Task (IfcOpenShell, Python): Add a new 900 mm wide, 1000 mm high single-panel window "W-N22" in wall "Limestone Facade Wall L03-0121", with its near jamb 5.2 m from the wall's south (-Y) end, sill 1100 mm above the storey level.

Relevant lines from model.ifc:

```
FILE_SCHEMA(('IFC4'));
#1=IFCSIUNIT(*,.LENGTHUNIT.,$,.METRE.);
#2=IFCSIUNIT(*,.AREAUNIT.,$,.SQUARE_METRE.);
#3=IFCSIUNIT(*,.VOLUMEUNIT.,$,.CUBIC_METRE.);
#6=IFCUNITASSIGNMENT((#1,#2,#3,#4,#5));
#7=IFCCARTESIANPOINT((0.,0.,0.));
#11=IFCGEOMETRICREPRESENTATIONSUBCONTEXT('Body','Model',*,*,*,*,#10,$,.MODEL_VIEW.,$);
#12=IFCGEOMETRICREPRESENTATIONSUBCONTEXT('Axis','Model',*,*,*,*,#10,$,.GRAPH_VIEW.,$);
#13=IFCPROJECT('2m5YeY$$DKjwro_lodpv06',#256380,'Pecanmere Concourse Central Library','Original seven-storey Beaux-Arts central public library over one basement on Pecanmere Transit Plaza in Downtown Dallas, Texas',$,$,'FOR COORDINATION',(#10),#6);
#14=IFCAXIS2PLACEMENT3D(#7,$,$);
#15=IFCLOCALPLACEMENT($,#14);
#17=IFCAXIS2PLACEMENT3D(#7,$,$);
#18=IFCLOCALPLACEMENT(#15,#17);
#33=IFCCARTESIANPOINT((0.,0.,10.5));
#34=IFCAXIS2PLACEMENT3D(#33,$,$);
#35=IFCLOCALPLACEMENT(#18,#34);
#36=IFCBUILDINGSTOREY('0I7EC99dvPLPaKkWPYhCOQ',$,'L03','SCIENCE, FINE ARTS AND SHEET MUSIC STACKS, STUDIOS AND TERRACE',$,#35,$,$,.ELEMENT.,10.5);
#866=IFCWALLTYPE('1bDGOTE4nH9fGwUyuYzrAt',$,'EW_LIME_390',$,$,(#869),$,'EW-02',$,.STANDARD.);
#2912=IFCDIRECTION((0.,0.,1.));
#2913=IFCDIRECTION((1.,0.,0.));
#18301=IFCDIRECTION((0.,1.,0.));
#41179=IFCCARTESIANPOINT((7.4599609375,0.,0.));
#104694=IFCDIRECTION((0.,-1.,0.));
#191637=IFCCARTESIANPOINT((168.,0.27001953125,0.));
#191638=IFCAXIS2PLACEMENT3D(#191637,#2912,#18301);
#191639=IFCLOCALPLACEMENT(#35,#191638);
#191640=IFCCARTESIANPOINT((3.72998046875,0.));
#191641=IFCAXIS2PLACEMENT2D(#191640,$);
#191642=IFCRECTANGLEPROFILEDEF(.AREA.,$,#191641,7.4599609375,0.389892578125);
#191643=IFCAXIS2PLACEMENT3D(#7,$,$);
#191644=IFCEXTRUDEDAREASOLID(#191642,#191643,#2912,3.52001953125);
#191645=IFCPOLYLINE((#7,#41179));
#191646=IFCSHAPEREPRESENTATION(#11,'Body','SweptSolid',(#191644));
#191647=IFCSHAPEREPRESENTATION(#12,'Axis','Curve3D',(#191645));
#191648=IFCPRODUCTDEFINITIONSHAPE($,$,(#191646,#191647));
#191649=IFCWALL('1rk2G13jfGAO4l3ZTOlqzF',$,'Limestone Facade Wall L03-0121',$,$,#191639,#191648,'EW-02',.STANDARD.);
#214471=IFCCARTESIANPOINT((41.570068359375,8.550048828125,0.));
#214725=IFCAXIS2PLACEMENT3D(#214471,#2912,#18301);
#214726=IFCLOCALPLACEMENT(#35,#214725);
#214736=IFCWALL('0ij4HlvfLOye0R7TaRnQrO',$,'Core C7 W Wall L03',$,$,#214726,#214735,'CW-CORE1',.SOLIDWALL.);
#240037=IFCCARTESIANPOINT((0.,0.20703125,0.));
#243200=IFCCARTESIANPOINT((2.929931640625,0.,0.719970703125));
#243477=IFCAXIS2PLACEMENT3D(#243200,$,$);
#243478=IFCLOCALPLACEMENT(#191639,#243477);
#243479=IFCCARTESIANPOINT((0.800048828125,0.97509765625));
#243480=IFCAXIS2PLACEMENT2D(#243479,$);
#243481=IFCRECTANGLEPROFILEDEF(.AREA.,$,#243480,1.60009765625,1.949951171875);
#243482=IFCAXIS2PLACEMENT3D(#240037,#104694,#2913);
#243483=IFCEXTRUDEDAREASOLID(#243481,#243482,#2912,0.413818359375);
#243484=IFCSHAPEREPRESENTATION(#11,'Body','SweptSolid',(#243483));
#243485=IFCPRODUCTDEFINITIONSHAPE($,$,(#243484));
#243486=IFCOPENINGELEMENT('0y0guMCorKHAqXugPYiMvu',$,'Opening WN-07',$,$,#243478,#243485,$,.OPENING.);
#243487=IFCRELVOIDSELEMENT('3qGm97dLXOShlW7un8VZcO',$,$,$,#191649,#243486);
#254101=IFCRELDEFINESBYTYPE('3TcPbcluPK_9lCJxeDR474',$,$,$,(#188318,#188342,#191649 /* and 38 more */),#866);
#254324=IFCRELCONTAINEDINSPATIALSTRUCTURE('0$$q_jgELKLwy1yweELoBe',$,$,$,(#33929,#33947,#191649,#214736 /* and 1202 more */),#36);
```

```python
import numpy as np
import ifcopenshell
import ifcopenshell.api.feature
import ifcopenshell.api.geometry
import ifcopenshell.api.root
import ifcopenshell.api.spatial
import ifcopenshell.geom
import ifcopenshell.util.element
import ifcopenshell.util.placement
import ifcopenshell.util.representation
import ifcopenshell.util.shape
import ifcopenshell.util.unit

model = ifcopenshell.open("model.ifc")
unit_scale = ifcopenshell.util.unit.calculate_unit_scale(model)
settings = ifcopenshell.geom.settings()


def volume(element):
    """Net volume in cubic metres, openings subtracted."""
    shape = ifcopenshell.geom.create_shape(settings, element)
    return ifcopenshell.util.shape.get_volume(shape.geometry)


wall = model.by_id(191649)
storey = ifcopenshell.util.element.get_container(wall, ifc_class="IfcBuildingStorey")
context = ifcopenshell.util.representation.get_context(model, "Model", "Body", "MODEL_VIEW")
before = volume(wall)

width, height, from_end, sill = 0.9, 1, 5.2, 1.1  # metres

# The wall runs along its own X axis, and the end named is its -X end.
wall_shape = ifcopenshell.geom.create_shape(settings, wall)
x, y, z = ifcopenshell.util.shape.get_vertices(wall_shape.geometry).T
start = x.min() + from_end
face, thickness = float(y.min()), float(y.max() - y.min())
wall_matrix = ifcopenshell.util.placement.get_local_placement(wall.ObjectPlacement)
level = ifcopenshell.util.placement.get_local_placement(storey.ObjectPlacement)[2, 3]


def in_wall(x, y):
    """Placement at x, y metres in the wall's axes, at sill height."""
    matrix = wall_matrix.copy()
    matrix[:, 3] = wall_matrix @ np.array([x / unit_scale, y / unit_scale, 0.0, 1.0])
    matrix[2, 3] = level + sill / unit_scale
    return matrix


# Opening: a box that overshoots both wall faces by 50 mm.
opening = ifcopenshell.api.root.create_entity(model, ifc_class="IfcOpeningElement", predefined_type="OPENING")
box = ifcopenshell.api.geometry.add_wall_representation(
    model, context=context, length=width, height=height, thickness=thickness + 0.1
)
ifcopenshell.api.geometry.assign_representation(model, product=opening, representation=box)
ifcopenshell.api.geometry.edit_object_placement(model, product=opening, matrix=in_wall(start, face - 0.05), is_si=False)
ifcopenshell.api.feature.add_feature(model, feature=opening, element=wall)

window = ifcopenshell.api.root.create_entity(model, ifc_class="IfcWindow", name="W-N22", predefined_type="WINDOW")
window.OverallWidth, window.OverallHeight = width / unit_scale, height / unit_scale
window.PartitioningType = "SINGLE_PANEL"
body = ifcopenshell.api.geometry.add_window_representation(
    model,
    context=context,
    overall_width=window.OverallWidth,
    overall_height=window.OverallHeight,
    partition_type="SINGLE_PANEL",
)
ifcopenshell.api.geometry.assign_representation(model, product=window, representation=body)
ifcopenshell.api.spatial.assign_container(model, products=[window], relating_structure=storey)
ifcopenshell.api.feature.add_filling(model, opening=opening, element=window)

# Centre the window in the wall's thickness.
ifcopenshell.api.geometry.edit_object_placement(model, product=window, matrix=in_wall(start, face), is_si=False)
window_shape = ifcopenshell.geom.create_shape(settings, window)
depth = ifcopenshell.util.shape.get_vertices(window_shape.geometry)[:, 1]
offset = face + thickness / 2 - (depth.min() + depth.max()) / 2
ifcopenshell.api.geometry.edit_object_placement(model, product=window, matrix=in_wall(start, offset), is_si=False)

after = volume(wall)

print(f"wall volume {before:.3f} -> {after:.3f} m3")

model.write("model-out.ifc")
```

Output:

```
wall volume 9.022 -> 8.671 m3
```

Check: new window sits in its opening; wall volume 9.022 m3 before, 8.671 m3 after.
